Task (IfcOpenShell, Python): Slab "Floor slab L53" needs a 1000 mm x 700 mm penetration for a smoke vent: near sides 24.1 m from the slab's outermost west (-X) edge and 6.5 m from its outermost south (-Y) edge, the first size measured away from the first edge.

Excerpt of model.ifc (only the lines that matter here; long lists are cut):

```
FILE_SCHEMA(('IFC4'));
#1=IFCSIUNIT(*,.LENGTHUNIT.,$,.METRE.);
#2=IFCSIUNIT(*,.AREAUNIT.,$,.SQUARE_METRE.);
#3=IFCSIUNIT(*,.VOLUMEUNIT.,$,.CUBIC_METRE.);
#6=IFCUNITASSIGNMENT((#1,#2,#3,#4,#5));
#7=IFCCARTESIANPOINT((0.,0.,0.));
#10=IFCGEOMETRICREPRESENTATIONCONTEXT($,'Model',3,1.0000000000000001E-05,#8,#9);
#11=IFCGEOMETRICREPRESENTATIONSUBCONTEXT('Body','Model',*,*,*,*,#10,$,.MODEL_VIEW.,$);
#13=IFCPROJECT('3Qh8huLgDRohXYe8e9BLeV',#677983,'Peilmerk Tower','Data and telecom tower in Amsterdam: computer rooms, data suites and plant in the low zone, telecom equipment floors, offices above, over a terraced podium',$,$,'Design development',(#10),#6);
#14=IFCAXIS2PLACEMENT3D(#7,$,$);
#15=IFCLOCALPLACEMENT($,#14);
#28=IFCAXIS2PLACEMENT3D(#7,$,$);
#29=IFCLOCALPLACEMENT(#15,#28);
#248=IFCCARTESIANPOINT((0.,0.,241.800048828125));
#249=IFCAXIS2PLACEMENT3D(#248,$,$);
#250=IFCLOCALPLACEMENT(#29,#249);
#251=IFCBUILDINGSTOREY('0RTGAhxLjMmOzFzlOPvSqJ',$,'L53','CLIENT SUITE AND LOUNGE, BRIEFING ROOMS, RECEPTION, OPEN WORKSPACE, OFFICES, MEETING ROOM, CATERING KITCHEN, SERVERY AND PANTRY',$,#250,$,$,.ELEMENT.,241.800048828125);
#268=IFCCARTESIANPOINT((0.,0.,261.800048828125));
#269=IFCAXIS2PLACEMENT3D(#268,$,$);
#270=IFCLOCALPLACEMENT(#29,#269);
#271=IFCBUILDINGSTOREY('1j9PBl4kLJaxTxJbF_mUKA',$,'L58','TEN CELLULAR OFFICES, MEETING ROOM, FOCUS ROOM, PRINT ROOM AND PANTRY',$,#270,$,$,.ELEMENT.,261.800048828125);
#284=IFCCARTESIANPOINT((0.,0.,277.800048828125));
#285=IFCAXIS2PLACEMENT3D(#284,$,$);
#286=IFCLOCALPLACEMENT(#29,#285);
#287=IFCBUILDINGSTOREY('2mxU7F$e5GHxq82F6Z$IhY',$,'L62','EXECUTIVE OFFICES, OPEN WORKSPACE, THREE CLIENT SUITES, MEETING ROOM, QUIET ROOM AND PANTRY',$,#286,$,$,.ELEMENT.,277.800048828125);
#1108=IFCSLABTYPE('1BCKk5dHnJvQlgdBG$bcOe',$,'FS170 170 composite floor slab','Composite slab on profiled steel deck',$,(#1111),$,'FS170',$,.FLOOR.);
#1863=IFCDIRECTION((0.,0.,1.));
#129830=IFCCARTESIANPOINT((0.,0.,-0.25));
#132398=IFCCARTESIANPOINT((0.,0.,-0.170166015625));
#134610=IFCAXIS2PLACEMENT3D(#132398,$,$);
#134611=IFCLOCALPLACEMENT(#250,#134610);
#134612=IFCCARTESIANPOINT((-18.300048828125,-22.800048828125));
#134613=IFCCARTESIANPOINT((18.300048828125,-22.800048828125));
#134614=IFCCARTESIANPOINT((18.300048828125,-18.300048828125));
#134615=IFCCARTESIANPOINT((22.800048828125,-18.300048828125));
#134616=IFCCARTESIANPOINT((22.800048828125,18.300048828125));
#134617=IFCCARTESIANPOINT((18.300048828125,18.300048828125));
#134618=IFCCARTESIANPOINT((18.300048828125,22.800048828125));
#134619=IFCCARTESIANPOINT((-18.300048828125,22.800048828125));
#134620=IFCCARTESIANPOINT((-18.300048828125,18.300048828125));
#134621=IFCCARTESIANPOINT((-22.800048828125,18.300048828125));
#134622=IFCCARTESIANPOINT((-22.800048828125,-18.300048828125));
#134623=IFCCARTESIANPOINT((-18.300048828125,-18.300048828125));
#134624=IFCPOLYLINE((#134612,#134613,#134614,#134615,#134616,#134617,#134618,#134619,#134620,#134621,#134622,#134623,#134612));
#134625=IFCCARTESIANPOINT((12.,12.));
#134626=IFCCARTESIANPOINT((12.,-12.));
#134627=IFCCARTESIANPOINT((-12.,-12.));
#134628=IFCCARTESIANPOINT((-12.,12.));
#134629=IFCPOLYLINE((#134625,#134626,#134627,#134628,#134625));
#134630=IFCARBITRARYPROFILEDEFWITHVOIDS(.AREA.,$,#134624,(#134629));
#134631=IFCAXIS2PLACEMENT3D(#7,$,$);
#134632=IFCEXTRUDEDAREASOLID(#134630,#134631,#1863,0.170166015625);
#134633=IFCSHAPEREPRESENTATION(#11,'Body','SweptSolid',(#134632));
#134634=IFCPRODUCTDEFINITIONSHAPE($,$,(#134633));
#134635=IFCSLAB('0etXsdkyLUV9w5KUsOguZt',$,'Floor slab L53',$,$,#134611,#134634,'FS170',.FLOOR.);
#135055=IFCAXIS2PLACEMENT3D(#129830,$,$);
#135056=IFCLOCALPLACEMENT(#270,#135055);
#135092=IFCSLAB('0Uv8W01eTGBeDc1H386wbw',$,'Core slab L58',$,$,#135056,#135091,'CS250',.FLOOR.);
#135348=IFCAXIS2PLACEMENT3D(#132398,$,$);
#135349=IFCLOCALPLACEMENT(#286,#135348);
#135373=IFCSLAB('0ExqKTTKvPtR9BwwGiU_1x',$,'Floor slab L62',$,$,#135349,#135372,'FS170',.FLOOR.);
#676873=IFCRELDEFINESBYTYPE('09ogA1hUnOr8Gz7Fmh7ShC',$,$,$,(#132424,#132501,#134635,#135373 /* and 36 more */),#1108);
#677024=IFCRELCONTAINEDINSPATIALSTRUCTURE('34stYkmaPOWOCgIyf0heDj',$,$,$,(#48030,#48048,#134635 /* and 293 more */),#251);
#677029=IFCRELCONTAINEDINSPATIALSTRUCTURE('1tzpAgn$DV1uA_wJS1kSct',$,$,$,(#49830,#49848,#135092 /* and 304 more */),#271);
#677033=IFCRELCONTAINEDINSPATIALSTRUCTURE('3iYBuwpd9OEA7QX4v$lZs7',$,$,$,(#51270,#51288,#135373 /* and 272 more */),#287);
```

```python
import numpy as np
import ifcopenshell
import ifcopenshell.api.feature
import ifcopenshell.api.geometry
import ifcopenshell.api.root
import ifcopenshell.geom
import ifcopenshell.util.placement
import ifcopenshell.util.representation
import ifcopenshell.util.shape
import ifcopenshell.util.unit

model = ifcopenshell.open("model.ifc")
unit_scale = ifcopenshell.util.unit.calculate_unit_scale(model)
settings = ifcopenshell.geom.settings()


def volume(element):
    """Net volume in cubic metres, openings subtracted."""
    shape = ifcopenshell.geom.create_shape(settings, element)
    return ifcopenshell.util.shape.get_volume(shape.geometry)


slab = model.by_guid("0etXsdkyLUV9w5KUsOguZt")
before = volume(slab)

# Extent in the slab's own axes, in metres. The edges named are its -X and -Y sides.
slab_shape = ifcopenshell.geom.create_shape(settings, slab)
vertices = ifcopenshell.util.shape.get_vertices(slab_shape.geometry)
x_min, y_min, bottom = vertices.min(axis=0)
top = vertices[:, 2].max()

opening = ifcopenshell.api.root.create_entity(model, ifc_class="IfcOpeningElement", name="Smoke vent opening", predefined_type="OPENING")
context = ifcopenshell.util.representation.get_context(model, "Model", "Body", "MODEL_VIEW")
width, depth = 1, 0.7
outline = [(0.0, 0.0), (width, 0.0), (width, depth), (0.0, depth), (0.0, 0.0)]
# Overshoot both faces by 50 mm so the cut is clean.
shape = ifcopenshell.api.geometry.add_slab_representation(
    model, context=context, depth=top - bottom + 0.1, polyline=outline
)
ifcopenshell.api.geometry.assign_representation(model, product=opening, representation=shape)

matrix = ifcopenshell.util.placement.get_local_placement(slab.ObjectPlacement)
matrix[:, 3] = matrix @ np.append(np.array([x_min + 24.1, y_min + 6.5, bottom - 0.05]) / unit_scale, 1.0)
ifcopenshell.api.geometry.edit_object_placement(model, product=opening, matrix=matrix, is_si=False)
ifcopenshell.api.feature.add_feature(model, feature=opening, element=slab)

after = volume(slab)

print(f"slab volume {before:.3f} -> {after:.3f} m3")

model.write("model-out.ifc")
```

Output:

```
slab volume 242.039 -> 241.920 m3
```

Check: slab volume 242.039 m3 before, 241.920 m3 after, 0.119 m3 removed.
